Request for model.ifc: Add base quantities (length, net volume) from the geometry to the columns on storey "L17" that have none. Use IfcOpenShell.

First a look at what the model holds.

```python
import ifcopenshell
import ifcopenshell.util.element
import ifcopenshell.util.unit

model = ifcopenshell.open("model.ifc")
print(model.schema)
for unit_type in ("LENGTHUNIT", "AREAUNIT", "VOLUMEUNIT"):
    print(unit_type, ifcopenshell.util.unit.calculate_unit_scale(model, unit_type))
storey = next(s for s in model.by_type("IfcBuildingStorey") if s.Name == "L17")
columns = [e for e in ifcopenshell.util.element.get_decomposition(storey) if e.is_a("IfcColumn")]
for e in sorted(columns, key=lambda e: e.id()):
    print(e.id(), e.is_a(), e.Name, list(ifcopenshell.util.element.get_psets(e, qtos_only=True)), sep=" | ")
```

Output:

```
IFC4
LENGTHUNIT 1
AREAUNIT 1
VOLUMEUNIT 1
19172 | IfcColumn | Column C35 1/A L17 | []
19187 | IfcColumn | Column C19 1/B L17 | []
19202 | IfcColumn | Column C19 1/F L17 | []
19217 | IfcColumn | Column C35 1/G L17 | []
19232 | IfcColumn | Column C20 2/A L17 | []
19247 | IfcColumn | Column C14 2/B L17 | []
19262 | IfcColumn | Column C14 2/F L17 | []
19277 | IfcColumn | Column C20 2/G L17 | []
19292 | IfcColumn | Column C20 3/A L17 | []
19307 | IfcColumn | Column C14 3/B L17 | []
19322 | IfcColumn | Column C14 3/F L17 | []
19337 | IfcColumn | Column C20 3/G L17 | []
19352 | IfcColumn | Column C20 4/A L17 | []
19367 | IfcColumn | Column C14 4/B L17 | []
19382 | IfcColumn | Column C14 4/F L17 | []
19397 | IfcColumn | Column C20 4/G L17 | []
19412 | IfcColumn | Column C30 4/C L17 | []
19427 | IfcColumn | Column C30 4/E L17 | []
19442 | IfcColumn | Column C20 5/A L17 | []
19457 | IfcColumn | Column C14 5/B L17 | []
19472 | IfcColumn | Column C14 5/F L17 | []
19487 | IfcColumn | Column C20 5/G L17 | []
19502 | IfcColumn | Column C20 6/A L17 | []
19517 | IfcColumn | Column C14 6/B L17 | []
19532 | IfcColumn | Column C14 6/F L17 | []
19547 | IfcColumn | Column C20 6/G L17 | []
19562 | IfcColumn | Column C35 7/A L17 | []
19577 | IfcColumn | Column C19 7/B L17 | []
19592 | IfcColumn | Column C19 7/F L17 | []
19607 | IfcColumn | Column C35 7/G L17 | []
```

```python
import ifcopenshell
import ifcopenshell.api.pset
import ifcopenshell.geom
import ifcopenshell.util.element
import ifcopenshell.util.shape
import ifcopenshell.util.unit

model = ifcopenshell.open("model.ifc")
unit_scale = ifcopenshell.util.unit.calculate_unit_scale(model)
volume_scale = ifcopenshell.util.unit.calculate_unit_scale(model, "VOLUMEUNIT")
settings = ifcopenshell.geom.settings()

storey = next(s for s in model.by_type("IfcBuildingStorey") if s.Name == "L17")
columns = [e for e in ifcopenshell.util.element.get_decomposition(storey) if e.is_a("IfcColumn")]

for e in sorted(columns, key=lambda e: e.id()):
    if ifcopenshell.util.element.get_psets(e, qtos_only=True, should_inherit=False):
        continue
    # Geometry comes back in metres, in the element's own axes.
    shape = ifcopenshell.geom.create_shape(settings, e)
    values = {
        "Length": ifcopenshell.util.shape.get_z(shape.geometry) / unit_scale,
        "NetVolume": ifcopenshell.util.shape.get_volume(shape.geometry) / volume_scale,
    }
    qto = ifcopenshell.api.pset.add_qto(model, product=e, name="Qto_ColumnBaseQuantities")
    ifcopenshell.api.pset.edit_qto(model, qto=qto, properties=values)
    print(e.id(), {k: round(v, 3) for k, v in values.items()})

model.write("model_edited.ifc")
```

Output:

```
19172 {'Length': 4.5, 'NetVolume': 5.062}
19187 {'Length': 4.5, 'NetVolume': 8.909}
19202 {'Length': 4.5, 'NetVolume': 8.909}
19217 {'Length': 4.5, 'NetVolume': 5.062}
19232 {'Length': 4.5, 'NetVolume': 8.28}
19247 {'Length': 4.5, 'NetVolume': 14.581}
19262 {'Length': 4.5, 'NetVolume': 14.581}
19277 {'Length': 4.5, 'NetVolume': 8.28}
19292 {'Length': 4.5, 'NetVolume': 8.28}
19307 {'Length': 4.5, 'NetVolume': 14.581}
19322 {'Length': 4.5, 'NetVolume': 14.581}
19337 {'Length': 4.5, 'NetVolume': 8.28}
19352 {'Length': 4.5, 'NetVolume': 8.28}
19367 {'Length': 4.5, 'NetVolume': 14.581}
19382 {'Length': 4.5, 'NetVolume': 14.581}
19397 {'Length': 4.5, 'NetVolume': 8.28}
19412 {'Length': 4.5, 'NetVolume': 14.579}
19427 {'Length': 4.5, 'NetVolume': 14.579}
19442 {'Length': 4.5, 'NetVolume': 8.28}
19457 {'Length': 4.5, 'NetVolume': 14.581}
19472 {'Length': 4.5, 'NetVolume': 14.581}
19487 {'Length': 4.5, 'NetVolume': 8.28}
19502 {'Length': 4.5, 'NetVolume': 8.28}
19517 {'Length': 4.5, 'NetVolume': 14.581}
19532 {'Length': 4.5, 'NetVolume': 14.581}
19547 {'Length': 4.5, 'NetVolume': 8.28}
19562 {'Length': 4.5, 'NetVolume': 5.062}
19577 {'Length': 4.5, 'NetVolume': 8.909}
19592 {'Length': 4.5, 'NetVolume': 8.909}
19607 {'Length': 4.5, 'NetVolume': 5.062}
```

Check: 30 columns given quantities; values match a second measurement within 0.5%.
